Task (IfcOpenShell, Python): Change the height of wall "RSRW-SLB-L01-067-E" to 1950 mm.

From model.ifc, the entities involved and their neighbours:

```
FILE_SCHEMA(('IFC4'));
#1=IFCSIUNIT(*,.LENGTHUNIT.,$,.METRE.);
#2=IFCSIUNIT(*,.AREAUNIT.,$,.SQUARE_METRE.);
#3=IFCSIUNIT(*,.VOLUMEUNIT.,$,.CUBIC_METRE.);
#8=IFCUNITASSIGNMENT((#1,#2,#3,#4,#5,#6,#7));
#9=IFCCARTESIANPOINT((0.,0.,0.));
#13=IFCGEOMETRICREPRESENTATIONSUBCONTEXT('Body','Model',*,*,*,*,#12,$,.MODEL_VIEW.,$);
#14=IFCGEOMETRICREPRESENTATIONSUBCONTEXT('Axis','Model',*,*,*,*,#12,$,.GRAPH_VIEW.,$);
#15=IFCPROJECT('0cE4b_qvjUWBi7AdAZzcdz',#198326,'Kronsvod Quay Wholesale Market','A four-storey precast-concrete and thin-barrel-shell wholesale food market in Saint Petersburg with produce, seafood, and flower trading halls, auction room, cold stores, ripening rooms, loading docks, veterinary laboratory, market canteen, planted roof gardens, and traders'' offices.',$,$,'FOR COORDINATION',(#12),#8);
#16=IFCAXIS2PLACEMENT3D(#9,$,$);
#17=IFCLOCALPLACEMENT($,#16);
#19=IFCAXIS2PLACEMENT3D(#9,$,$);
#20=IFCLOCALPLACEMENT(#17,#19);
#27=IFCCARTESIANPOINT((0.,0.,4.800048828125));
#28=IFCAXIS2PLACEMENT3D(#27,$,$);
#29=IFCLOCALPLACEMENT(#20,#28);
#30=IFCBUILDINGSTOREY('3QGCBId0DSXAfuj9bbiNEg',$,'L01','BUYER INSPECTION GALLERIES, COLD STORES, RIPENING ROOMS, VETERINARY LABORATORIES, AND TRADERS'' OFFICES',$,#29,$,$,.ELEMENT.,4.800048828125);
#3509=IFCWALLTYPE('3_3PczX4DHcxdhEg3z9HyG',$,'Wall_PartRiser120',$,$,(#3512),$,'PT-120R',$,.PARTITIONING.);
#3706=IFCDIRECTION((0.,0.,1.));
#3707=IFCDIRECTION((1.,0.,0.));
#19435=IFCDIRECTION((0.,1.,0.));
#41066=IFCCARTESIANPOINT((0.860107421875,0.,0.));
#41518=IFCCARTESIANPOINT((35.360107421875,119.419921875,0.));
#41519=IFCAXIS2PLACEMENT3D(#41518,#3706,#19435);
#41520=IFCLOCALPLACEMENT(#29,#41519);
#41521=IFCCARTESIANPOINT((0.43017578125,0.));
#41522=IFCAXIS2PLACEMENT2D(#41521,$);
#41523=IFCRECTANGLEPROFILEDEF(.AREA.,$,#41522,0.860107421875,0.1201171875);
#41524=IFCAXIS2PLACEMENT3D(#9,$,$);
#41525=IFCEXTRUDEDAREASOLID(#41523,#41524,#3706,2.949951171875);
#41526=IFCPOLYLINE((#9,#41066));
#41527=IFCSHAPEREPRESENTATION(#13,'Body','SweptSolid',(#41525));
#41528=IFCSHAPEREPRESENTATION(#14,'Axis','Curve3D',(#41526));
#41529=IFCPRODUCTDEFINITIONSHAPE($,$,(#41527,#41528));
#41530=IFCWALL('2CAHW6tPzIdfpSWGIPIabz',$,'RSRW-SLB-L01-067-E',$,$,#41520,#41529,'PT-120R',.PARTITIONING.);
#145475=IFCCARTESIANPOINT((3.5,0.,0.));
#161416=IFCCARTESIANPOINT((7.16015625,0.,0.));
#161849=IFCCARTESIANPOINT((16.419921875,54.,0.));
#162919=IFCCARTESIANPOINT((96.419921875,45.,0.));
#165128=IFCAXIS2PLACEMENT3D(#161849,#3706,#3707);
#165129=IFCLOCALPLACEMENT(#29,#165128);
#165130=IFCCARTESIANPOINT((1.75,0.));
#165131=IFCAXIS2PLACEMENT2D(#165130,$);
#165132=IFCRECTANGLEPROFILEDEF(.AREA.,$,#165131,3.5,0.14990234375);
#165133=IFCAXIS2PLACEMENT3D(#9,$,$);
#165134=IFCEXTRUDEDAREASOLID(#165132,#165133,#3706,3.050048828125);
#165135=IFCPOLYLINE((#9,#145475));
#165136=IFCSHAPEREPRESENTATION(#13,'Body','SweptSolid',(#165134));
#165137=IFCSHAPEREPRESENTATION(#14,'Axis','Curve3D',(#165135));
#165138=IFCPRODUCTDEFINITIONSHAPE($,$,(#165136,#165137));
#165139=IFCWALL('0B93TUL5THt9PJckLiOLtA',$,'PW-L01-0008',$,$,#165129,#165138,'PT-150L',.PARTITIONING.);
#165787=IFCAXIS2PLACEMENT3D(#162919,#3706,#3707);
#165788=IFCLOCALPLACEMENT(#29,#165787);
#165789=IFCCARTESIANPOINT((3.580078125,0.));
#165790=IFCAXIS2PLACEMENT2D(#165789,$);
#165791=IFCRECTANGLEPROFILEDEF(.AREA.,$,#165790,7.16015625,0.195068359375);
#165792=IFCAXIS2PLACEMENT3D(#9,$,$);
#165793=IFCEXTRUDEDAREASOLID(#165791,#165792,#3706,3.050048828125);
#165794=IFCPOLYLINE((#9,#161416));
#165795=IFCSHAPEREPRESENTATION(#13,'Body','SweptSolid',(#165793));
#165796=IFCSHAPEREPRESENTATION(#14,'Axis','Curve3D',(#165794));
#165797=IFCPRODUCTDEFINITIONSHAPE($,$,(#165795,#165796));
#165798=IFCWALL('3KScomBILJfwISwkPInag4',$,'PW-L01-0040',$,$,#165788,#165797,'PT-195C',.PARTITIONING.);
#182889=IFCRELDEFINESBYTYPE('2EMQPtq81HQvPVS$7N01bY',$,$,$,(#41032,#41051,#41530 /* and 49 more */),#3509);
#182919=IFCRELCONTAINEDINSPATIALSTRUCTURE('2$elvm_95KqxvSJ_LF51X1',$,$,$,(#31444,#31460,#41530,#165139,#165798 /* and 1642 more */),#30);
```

```python
import ifcopenshell
import ifcopenshell.geom
import ifcopenshell.util.representation
import ifcopenshell.util.shape

model = ifcopenshell.open("model.ifc")
settings = ifcopenshell.geom.settings()


def volume(element):
    """Net volume in cubic metres, openings subtracted."""
    shape = ifcopenshell.geom.create_shape(settings, element)
    return ifcopenshell.util.shape.get_volume(shape.geometry)


wall = model.by_guid("2CAHW6tPzIdfpSWGIPIabz")
before = volume(wall)

body = ifcopenshell.util.representation.get_representation(wall, "Model", "Body")
solid = body.Items[0]
old_height = solid.Depth
solid.Depth = 1.95
after = volume(wall)

print(f"height {old_height:g} -> {solid.Depth:g}, volume {before:.3f} -> {after:.3f} m3")

model.write("model_edited.ifc")
```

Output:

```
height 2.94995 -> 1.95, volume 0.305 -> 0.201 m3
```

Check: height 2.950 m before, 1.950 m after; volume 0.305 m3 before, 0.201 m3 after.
